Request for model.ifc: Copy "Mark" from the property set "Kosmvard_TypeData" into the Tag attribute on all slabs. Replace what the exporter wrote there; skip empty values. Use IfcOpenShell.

First a look at what the model holds.

```python
import ifcopenshell
import ifcopenshell.util.element

model = ifcopenshell.open("model.ifc")
print(model.schema)
slabs = model.by_type("IfcSlab")
print(len(slabs), "slabs")
for e in slabs[:8]:
    source = ifcopenshell.util.element.get_pset(e, "Kosmvard_TypeData", "Mark")
    target = e.Tag
    print(e.id(), repr(source), repr(target), sep=" | ")
```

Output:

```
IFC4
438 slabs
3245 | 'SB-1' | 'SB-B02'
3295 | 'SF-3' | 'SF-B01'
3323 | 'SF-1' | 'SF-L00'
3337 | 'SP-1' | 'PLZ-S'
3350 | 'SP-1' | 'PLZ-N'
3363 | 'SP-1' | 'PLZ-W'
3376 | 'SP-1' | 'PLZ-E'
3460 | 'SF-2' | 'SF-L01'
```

```python
import ifcopenshell
import ifcopenshell.util.element

model = ifcopenshell.open("model.ifc")

count = 0
for e in model.by_type("IfcSlab"):
    value = ifcopenshell.util.element.get_pset(e, "Kosmvard_TypeData", "Mark")
    current = e.Tag
    if not value or not value.strip() or current == value:
        continue
    e.Tag = value
    count += 1

print(count, "slabs updated")

model.write("model_updated.ifc")
```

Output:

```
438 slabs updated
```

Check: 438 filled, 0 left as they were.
